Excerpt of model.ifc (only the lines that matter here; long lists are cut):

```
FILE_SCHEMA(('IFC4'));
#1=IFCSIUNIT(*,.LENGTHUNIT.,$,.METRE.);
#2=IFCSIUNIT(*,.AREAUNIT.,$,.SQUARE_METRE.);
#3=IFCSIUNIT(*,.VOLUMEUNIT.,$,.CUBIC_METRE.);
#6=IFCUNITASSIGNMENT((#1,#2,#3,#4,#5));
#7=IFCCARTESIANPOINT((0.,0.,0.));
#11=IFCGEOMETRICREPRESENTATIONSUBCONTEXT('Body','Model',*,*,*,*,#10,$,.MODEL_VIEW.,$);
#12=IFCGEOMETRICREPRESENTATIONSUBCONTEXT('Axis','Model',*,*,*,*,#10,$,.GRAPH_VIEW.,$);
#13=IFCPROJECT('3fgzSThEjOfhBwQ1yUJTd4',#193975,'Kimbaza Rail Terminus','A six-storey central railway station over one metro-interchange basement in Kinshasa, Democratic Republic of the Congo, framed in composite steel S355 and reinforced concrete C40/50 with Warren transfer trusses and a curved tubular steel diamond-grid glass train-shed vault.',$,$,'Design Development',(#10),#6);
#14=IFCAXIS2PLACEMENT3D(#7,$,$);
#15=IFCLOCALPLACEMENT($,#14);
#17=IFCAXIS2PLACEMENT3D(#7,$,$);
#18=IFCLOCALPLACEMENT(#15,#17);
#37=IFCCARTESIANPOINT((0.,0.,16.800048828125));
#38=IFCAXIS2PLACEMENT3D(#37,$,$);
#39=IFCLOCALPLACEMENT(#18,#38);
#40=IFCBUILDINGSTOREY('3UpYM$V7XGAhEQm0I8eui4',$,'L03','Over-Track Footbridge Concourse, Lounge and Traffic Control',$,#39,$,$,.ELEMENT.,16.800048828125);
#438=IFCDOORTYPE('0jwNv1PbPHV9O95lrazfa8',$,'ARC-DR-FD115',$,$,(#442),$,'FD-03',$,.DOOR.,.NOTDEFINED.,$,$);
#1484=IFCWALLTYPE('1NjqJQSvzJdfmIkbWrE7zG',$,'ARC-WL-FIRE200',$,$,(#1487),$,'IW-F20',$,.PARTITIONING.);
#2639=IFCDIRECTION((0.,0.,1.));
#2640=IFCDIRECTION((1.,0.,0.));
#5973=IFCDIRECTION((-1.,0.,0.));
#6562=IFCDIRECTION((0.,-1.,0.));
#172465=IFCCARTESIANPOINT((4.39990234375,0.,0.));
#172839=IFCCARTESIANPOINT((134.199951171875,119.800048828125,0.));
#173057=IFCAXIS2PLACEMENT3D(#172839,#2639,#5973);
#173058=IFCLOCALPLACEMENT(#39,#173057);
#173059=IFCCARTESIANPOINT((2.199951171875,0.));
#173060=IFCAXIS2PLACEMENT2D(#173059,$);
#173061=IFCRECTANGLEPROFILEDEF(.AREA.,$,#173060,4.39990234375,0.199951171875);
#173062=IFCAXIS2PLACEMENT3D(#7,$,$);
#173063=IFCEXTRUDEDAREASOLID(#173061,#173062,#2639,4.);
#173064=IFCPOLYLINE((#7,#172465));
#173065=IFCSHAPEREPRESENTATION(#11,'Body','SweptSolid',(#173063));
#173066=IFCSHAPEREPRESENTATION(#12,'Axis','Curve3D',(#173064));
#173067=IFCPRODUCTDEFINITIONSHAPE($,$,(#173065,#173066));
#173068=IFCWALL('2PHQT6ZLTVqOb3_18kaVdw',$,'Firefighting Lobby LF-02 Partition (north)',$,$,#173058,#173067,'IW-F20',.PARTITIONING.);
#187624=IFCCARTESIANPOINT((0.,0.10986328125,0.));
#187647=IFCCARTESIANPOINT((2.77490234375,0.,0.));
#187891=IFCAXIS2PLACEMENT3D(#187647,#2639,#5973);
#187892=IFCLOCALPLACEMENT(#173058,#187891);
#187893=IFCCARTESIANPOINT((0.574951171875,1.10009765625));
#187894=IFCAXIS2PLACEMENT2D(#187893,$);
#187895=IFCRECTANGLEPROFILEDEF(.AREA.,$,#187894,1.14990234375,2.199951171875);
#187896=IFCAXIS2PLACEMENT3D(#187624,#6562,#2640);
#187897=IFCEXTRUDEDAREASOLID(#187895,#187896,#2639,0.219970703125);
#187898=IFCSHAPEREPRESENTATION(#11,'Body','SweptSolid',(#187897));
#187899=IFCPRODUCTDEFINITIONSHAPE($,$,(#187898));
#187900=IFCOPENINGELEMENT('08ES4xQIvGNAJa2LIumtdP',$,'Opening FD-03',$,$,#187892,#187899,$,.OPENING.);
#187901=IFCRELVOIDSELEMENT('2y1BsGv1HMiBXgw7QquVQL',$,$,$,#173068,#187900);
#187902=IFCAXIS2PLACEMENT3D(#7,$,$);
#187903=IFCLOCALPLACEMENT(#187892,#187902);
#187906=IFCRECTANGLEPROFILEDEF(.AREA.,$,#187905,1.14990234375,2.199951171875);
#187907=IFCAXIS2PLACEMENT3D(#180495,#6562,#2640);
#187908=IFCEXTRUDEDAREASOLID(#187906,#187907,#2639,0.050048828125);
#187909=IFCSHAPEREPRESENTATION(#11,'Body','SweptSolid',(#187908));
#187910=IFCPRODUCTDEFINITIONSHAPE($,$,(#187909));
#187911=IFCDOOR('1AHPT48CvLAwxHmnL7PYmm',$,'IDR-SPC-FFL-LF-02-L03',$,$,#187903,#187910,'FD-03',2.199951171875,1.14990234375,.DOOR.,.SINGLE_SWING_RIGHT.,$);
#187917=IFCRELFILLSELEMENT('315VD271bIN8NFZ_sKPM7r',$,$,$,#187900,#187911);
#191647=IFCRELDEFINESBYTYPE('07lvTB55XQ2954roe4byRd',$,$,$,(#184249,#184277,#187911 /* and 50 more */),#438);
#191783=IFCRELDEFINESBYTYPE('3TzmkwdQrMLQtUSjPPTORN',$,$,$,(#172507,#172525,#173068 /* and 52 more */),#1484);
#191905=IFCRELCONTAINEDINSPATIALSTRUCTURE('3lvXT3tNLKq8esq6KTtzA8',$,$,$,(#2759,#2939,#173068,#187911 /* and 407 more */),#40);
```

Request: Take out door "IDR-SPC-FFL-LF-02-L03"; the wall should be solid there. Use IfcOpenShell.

```python
import ifcopenshell
import ifcopenshell.api.feature
import ifcopenshell.api.root
import ifcopenshell.geom
import ifcopenshell.util.shape

model = ifcopenshell.open("model.ifc")
settings = ifcopenshell.geom.settings()


def volume(element):
    """Net volume in cubic metres, openings subtracted."""
    shape = ifcopenshell.geom.create_shape(settings, element)
    return ifcopenshell.util.shape.get_volume(shape.geometry)


door = model.by_guid("1AHPT48CvLAwxHmnL7PYmm")
opening = door.FillsVoids[0].RelatingOpeningElement
wall = opening.VoidsElements[0].RelatingBuildingElement
before = volume(wall)

ifcopenshell.api.root.remove_product(model, product=door)
ifcopenshell.api.feature.remove_feature(model, feature=opening)

after = volume(wall)

print(f"wall volume {before:.3f} -> {after:.3f} m3")

model.write("model_rev.ifc")
```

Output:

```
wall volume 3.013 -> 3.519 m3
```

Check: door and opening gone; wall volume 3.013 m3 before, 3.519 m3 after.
